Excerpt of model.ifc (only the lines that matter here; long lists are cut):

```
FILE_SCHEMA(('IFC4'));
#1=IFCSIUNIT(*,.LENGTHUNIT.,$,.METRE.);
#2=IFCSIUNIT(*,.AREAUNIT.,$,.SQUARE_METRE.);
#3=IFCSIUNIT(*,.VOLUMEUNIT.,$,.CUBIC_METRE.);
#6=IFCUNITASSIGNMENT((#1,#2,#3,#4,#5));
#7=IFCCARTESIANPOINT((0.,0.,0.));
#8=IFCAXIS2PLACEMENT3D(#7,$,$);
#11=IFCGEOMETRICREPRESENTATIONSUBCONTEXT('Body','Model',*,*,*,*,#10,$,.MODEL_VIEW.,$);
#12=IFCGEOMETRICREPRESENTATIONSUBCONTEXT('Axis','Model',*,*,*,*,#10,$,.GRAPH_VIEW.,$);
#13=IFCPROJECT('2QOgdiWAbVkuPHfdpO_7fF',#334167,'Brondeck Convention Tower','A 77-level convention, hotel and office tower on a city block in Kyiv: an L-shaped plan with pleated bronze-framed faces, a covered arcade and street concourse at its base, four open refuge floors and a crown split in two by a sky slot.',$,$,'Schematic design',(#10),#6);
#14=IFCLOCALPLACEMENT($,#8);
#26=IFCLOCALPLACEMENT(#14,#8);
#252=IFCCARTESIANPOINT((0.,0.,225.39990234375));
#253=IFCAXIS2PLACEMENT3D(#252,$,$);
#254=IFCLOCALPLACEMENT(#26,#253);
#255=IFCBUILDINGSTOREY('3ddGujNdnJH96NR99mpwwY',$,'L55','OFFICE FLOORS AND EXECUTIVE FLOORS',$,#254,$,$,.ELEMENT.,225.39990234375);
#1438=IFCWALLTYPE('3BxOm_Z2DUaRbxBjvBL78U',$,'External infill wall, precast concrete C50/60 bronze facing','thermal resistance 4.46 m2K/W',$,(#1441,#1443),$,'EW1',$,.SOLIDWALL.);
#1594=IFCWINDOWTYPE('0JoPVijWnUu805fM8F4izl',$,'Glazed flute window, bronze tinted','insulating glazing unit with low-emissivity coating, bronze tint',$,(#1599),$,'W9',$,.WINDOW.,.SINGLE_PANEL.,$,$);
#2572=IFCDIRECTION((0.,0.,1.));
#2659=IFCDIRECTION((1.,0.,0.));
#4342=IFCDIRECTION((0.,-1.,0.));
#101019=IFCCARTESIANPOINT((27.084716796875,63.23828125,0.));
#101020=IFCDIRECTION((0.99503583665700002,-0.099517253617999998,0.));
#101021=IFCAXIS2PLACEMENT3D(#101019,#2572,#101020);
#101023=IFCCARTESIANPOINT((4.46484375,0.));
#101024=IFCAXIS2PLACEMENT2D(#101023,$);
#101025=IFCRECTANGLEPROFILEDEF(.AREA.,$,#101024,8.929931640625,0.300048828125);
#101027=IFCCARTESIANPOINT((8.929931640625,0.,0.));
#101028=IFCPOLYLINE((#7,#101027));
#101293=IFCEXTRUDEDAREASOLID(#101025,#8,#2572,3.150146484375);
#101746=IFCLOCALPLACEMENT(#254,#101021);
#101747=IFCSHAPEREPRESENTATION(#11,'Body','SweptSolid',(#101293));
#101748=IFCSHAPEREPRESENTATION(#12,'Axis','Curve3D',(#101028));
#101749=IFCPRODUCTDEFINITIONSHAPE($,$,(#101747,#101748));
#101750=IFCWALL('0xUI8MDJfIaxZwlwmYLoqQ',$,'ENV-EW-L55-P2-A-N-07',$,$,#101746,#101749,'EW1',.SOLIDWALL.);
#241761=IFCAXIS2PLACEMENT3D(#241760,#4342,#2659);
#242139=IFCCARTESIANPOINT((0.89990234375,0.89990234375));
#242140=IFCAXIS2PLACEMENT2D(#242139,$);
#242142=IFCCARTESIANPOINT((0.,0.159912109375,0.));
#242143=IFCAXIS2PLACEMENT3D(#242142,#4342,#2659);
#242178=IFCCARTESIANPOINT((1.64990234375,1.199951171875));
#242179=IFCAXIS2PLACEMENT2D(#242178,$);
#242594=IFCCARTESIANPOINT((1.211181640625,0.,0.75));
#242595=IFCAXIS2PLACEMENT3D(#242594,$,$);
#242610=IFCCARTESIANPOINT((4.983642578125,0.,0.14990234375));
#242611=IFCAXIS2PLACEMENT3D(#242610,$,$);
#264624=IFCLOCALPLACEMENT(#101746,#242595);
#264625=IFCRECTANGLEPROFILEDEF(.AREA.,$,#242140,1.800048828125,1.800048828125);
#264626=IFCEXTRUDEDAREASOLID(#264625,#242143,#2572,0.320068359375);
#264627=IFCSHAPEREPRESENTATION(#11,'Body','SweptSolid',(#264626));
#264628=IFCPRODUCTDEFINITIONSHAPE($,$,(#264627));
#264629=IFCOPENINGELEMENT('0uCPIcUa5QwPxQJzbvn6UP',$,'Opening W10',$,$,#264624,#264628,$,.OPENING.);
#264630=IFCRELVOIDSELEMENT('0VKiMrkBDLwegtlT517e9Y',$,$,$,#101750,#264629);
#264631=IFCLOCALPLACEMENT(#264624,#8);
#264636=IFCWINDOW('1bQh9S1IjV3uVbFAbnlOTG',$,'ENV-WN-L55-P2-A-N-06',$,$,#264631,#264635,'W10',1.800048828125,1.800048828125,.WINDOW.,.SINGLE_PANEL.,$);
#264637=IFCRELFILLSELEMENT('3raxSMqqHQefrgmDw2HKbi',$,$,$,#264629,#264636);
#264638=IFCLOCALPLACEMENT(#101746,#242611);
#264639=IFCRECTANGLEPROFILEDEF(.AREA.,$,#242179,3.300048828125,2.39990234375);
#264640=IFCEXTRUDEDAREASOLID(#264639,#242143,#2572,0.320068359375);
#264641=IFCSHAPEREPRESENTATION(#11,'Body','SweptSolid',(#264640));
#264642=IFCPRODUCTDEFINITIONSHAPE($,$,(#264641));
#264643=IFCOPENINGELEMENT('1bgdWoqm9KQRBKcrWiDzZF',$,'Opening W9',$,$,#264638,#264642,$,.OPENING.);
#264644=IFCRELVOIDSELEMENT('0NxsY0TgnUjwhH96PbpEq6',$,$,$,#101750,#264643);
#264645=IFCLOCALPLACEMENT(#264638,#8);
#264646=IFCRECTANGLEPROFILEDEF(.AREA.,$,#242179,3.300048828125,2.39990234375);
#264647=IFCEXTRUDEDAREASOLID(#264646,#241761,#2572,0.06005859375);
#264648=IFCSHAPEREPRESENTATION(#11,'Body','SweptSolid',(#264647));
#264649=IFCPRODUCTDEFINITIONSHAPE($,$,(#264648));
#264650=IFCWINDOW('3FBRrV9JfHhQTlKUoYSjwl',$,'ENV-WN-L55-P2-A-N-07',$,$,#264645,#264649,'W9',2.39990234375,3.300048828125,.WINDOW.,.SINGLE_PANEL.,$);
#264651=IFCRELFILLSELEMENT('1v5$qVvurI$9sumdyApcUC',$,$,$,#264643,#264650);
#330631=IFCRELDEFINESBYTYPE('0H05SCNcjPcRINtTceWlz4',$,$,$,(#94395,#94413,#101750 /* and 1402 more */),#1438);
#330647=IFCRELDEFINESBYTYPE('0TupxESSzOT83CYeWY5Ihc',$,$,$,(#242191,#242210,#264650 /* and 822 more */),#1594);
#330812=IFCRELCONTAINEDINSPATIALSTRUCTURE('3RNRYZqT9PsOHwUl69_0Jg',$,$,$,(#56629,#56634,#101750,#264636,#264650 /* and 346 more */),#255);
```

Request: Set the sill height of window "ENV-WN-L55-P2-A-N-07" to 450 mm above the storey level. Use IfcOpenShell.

```python
import numpy as np
import ifcopenshell
import ifcopenshell.api.geometry
import ifcopenshell.geom
import ifcopenshell.util.element
import ifcopenshell.util.placement
import ifcopenshell.util.shape
import ifcopenshell.util.unit

model = ifcopenshell.open("model.ifc")
unit_scale = ifcopenshell.util.unit.calculate_unit_scale(model)

window = model.by_id(264650)
opening = window.FillsVoids[0].RelatingOpeningElement
storey = ifcopenshell.util.element.get_container(window, ifc_class="IfcBuildingStorey")
level = ifcopenshell.util.placement.get_local_placement(storey.ObjectPlacement)[2, 3]

# The opening's origin need not be at the sill, so measure its lowest point.
shape = ifcopenshell.geom.create_shape(ifcopenshell.geom.settings(), opening)
bottom = ifcopenshell.util.shape.get_shape_bottom_elevation(shape, shape.geometry) / unit_scale
dz = level + 0.45 / unit_scale - bottom

shift = np.array([0.0, 0.0, dz])
# The window is placed relative to its opening, so it follows when the opening moves.
matrix = ifcopenshell.util.placement.get_local_placement(opening.ObjectPlacement)
matrix[:3, 3] += shift
ifcopenshell.api.geometry.edit_object_placement(
    model, product=opening, matrix=matrix, is_si=False, should_transform_children=True
)

print(f"moved by {dz * unit_scale:+.3f} m")

model.write("model-out.ifc")
```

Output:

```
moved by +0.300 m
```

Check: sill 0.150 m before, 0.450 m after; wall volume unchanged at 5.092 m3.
